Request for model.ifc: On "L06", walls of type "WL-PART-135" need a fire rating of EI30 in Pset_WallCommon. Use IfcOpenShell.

First a look at what the model holds.

```python
import ifcopenshell
import ifcopenshell.util.element

model = ifcopenshell.open("model.ifc")
print(model.schema)
storey = next(s for s in model.by_type("IfcBuildingStorey") if s.Name == "L06")
walls = [e for e in ifcopenshell.util.element.get_decomposition(storey) if e.is_a("IfcWall")]
seen = {}
for e in walls:
    element_type = ifcopenshell.util.element.get_type(e)
    key = (element_type.Name if element_type != e and element_type else None, ifcopenshell.util.element.get_pset(e, "Pset_WallCommon", "FireRating"))
    seen[key] = seen.get(key, 0) + 1
for (name, value), count in sorted(seen.items(), key=str):
    print(count, "x", name, "|", value)
```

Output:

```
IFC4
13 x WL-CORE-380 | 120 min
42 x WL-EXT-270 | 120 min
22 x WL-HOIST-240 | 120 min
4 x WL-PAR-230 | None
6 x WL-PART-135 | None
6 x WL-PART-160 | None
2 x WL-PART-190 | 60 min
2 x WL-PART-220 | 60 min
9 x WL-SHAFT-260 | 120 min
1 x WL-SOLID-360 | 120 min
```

```python
import ifcopenshell
import ifcopenshell.api.pset
import ifcopenshell.util.element

model = ifcopenshell.open("model.ifc")

storey = next(s for s in model.by_type("IfcBuildingStorey") if s.Name == "L06")
walls = [e for e in ifcopenshell.util.element.get_decomposition(storey) if e.is_a("IfcWall")]

count = 0
for e in walls:
    element_type = ifcopenshell.util.element.get_type(e)
    if element_type in (None, e) or element_type.Name != "WL-PART-135":
        continue
    # add_pset returns the element's existing set when there is one.
    pset = ifcopenshell.api.pset.add_pset(model, product=e, name="Pset_WallCommon")
    ifcopenshell.api.pset.edit_pset(model, pset=pset, properties={"FireRating": "EI30"})
    count += 1

print(count, "walls updated")

model.write("model_v2.ifc")
```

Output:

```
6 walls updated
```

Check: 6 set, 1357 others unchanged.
